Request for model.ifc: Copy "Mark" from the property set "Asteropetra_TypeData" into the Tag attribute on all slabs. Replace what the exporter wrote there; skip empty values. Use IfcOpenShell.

First a look at what the model holds.

```python
import ifcopenshell
import ifcopenshell.util.element

model = ifcopenshell.open("model.ifc")
print(model.schema)
slabs = model.by_type("IfcSlab")
print(len(slabs), "slabs")
for e in slabs[:8]:
    source = ifcopenshell.util.element.get_pset(e, "Asteropetra_TypeData", "Mark")
    target = e.Tag
    print(e.id(), repr(source), repr(target), sep=" | ")
```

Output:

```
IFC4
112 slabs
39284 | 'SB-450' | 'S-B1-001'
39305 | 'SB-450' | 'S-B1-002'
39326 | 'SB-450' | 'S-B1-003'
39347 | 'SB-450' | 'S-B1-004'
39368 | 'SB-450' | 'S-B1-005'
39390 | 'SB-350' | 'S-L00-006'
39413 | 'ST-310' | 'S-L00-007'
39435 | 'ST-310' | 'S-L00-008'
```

```python
import ifcopenshell
import ifcopenshell.util.element

model = ifcopenshell.open("model.ifc")

count = 0
for e in model.by_type("IfcSlab"):
    value = ifcopenshell.util.element.get_pset(e, "Asteropetra_TypeData", "Mark")
    current = e.Tag
    if not value or not value.strip() or current == value:
        continue
    e.Tag = value
    count += 1

print(count, "slabs updated")

model.write("model_updated.ifc")
```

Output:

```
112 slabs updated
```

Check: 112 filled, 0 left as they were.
